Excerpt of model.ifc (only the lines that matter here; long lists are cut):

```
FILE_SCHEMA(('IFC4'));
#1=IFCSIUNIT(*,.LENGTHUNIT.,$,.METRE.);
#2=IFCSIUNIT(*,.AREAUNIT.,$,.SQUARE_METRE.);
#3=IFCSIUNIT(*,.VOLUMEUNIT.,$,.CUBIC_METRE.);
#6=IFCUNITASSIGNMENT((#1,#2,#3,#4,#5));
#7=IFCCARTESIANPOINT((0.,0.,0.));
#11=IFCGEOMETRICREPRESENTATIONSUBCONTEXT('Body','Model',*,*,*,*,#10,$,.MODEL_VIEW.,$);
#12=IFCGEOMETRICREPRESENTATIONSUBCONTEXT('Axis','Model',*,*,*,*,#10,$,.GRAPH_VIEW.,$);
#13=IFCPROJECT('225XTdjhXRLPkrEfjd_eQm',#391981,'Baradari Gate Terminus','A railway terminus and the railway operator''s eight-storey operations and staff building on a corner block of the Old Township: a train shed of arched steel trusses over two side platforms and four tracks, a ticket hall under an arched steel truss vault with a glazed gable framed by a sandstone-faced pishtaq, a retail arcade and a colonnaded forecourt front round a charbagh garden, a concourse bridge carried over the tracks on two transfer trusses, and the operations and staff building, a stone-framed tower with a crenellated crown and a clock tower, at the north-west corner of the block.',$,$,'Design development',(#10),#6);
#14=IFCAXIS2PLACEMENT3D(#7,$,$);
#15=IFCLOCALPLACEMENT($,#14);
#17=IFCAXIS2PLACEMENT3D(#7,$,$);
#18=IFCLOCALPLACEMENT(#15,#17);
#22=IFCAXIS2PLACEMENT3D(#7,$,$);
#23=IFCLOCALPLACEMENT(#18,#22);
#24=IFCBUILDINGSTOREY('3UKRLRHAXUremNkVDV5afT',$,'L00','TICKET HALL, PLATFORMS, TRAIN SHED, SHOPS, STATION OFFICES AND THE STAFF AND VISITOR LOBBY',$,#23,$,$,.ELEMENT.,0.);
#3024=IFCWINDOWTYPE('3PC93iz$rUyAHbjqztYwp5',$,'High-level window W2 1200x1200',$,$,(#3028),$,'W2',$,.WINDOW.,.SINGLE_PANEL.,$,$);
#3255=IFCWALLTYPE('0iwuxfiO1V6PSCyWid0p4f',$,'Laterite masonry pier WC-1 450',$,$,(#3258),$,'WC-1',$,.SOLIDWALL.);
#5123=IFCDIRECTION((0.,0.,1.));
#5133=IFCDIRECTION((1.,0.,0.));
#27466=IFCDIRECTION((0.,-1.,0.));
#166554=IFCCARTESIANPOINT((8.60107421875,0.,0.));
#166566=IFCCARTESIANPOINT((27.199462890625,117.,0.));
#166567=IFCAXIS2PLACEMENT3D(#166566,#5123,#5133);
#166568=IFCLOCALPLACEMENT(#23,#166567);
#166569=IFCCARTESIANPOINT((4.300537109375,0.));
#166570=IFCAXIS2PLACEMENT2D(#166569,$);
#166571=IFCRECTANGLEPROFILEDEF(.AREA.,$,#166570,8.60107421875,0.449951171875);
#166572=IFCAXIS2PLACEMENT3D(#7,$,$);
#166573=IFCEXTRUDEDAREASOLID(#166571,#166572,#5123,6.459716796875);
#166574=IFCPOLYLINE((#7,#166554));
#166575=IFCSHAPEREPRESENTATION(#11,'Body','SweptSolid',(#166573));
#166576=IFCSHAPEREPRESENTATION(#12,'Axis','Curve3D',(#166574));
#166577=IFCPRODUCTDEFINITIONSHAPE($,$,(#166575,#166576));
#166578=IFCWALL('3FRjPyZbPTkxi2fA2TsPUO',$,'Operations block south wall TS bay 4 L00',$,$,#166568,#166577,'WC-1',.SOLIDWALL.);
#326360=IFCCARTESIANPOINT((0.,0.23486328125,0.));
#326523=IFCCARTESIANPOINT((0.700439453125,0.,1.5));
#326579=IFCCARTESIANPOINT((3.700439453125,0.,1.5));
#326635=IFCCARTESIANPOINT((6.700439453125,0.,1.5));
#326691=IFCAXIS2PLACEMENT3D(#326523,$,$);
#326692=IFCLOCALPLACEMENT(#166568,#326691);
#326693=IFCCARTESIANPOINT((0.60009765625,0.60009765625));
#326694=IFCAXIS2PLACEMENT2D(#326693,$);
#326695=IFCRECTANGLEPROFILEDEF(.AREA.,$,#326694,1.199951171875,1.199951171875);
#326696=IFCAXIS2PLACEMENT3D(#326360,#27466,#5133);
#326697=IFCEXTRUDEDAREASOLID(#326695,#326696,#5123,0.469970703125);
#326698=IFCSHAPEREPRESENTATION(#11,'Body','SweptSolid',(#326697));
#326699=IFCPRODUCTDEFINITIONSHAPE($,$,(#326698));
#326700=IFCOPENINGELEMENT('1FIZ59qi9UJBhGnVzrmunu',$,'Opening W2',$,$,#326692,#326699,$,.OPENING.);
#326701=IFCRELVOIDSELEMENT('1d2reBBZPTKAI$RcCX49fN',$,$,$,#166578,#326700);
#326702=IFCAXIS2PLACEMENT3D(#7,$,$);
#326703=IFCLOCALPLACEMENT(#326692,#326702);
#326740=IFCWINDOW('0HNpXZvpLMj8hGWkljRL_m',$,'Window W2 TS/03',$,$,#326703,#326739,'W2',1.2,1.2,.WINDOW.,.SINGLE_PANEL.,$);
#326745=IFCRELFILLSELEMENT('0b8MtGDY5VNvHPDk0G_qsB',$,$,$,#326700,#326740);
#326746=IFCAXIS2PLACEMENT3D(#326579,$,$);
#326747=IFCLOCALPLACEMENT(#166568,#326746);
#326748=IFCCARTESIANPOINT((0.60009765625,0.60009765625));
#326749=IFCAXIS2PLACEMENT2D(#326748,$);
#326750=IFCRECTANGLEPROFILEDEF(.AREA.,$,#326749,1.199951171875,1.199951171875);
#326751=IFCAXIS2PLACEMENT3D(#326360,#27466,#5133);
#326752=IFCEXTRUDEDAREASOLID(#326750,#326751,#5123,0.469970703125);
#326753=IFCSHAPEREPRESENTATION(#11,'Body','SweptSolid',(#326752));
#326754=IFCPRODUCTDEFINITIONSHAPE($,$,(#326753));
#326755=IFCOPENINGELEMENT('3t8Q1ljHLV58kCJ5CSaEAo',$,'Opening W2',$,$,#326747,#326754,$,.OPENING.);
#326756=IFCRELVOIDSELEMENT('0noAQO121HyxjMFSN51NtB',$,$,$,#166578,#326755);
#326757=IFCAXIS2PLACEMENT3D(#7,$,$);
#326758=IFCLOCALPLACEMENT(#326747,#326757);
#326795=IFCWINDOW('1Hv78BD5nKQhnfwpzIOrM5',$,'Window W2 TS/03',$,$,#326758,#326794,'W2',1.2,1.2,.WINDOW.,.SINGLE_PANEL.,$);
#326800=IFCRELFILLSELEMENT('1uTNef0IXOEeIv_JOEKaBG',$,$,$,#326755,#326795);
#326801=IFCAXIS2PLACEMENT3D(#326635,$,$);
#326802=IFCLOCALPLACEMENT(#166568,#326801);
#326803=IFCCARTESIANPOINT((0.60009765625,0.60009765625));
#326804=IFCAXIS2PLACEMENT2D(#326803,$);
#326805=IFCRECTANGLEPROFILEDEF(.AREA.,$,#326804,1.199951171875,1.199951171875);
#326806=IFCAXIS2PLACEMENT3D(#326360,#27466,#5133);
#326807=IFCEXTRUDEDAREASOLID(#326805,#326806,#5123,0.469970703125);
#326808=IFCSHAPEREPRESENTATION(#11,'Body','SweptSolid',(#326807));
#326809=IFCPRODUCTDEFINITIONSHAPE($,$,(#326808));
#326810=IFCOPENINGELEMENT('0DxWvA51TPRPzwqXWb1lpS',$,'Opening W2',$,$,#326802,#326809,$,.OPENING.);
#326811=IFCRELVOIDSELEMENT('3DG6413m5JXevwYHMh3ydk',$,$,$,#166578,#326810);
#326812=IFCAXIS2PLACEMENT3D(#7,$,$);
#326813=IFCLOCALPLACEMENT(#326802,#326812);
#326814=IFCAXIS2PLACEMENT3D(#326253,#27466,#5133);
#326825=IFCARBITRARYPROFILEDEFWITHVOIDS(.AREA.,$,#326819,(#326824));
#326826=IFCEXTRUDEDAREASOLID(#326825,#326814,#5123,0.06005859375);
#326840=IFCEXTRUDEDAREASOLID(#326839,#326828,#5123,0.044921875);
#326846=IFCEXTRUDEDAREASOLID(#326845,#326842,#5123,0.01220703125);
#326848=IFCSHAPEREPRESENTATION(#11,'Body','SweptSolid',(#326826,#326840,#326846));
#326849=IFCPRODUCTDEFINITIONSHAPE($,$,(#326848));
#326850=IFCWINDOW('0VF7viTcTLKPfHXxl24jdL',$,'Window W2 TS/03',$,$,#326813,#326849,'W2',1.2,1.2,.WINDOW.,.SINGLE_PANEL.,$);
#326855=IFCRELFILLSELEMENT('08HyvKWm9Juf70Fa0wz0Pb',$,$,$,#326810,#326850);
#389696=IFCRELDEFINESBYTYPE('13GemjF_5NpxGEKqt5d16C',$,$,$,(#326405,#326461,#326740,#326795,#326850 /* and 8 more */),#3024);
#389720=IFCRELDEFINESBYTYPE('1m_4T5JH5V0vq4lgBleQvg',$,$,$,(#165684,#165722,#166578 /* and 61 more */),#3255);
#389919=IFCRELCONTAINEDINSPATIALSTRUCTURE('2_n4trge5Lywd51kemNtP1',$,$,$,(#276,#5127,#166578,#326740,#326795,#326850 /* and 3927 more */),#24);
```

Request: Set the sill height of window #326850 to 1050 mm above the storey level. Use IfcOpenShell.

```python
import numpy as np
import ifcopenshell
import ifcopenshell.api.geometry
import ifcopenshell.geom
import ifcopenshell.util.element
import ifcopenshell.util.placement
import ifcopenshell.util.shape
import ifcopenshell.util.unit

model = ifcopenshell.open("model.ifc")
unit_scale = ifcopenshell.util.unit.calculate_unit_scale(model)

window = model.by_id(326850)
opening = window.FillsVoids[0].RelatingOpeningElement
storey = ifcopenshell.util.element.get_container(window, ifc_class="IfcBuildingStorey")
level = ifcopenshell.util.placement.get_local_placement(storey.ObjectPlacement)[2, 3]

# The opening's origin need not be at the sill, so measure its lowest point.
shape = ifcopenshell.geom.create_shape(ifcopenshell.geom.settings(), opening)
bottom = ifcopenshell.util.shape.get_shape_bottom_elevation(shape, shape.geometry) / unit_scale
dz = level + 1.05 - bottom

shift = np.array([0.0, 0.0, dz])
# The window is placed relative to its opening, so it follows when the opening moves.
matrix = ifcopenshell.util.placement.get_local_placement(opening.ObjectPlacement)
matrix[:3, 3] += shift
ifcopenshell.api.geometry.edit_object_placement(
    model, product=opening, matrix=matrix, is_si=False, should_transform_children=True
)

print(f"moved by {dz * unit_scale:+.3f} m")

model.write("model_v2.ifc")
```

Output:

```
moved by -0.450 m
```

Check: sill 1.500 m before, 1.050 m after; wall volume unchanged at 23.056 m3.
